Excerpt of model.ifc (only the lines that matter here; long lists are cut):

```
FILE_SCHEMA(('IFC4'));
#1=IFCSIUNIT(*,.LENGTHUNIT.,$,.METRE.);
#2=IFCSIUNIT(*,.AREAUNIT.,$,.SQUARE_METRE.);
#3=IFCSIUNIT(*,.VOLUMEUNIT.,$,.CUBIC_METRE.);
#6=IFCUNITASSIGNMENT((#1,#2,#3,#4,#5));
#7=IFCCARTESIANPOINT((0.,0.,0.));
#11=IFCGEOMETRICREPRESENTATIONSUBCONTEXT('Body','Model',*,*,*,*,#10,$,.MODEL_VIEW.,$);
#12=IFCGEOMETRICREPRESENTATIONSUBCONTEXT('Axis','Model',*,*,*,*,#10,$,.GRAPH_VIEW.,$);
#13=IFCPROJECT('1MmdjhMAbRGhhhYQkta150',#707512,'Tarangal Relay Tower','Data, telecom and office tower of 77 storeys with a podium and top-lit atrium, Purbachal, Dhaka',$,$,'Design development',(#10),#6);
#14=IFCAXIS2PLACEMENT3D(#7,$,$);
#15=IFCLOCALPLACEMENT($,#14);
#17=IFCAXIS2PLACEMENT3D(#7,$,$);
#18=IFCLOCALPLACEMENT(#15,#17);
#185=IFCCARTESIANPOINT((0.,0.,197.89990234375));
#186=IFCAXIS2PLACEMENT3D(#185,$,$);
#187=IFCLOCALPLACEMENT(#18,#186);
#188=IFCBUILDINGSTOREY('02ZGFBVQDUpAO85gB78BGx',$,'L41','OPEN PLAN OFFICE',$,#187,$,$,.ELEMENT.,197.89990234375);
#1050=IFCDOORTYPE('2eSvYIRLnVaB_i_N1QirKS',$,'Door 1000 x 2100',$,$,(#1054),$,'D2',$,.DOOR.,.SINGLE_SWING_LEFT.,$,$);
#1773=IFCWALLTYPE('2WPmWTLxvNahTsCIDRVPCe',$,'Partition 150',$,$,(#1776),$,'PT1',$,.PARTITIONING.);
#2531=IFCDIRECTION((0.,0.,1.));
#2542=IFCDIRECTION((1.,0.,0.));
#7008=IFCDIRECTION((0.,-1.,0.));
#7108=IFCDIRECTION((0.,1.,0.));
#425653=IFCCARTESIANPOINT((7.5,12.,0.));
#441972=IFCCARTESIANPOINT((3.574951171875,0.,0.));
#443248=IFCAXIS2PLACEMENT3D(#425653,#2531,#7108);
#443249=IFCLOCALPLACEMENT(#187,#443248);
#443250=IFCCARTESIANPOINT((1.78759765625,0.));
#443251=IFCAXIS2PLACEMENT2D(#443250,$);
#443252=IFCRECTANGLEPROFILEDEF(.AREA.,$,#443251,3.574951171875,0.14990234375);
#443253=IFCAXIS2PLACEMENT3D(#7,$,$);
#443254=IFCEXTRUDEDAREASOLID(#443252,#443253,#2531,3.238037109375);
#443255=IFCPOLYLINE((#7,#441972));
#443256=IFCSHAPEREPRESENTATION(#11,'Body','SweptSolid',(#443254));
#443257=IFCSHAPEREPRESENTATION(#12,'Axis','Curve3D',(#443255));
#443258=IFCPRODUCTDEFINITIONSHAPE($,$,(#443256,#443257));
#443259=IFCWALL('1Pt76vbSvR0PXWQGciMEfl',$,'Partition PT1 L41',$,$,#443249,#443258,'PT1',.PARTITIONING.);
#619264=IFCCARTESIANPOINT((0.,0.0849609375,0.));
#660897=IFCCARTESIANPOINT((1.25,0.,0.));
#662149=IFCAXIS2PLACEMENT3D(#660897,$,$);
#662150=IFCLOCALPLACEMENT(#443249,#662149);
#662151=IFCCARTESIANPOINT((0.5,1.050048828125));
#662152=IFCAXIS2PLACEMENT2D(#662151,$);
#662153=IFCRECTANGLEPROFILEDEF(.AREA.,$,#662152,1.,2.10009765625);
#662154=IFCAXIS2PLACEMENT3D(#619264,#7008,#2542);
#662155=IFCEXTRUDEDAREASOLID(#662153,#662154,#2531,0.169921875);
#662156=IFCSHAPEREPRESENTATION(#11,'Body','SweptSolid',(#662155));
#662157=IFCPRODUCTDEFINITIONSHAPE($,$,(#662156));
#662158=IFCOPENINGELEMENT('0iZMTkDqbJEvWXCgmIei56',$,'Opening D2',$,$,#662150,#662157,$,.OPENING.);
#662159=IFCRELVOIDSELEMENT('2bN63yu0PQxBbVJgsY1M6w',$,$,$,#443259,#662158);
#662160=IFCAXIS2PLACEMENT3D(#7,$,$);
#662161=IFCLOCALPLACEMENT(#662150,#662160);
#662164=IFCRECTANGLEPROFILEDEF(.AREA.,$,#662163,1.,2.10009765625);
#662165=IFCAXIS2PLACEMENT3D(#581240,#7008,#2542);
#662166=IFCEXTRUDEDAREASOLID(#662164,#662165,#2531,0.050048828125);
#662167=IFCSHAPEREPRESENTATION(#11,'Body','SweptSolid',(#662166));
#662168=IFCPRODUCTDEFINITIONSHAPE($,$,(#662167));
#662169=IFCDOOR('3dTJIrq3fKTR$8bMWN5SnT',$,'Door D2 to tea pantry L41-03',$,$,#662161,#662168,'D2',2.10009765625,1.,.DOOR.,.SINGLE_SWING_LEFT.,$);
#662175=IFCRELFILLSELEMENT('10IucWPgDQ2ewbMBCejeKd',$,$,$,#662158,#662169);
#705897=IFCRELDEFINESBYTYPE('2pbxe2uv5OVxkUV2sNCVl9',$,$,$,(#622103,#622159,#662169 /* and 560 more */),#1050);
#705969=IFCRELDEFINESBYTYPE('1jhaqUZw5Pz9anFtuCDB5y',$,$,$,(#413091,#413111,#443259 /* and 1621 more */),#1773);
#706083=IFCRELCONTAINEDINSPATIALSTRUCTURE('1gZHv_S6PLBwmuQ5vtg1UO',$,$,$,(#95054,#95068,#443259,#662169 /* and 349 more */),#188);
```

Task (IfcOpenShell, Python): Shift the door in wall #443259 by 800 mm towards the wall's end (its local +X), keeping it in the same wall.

```python
import ifcopenshell
import ifcopenshell.api.geometry
import ifcopenshell.util.placement
import ifcopenshell.util.unit

model = ifcopenshell.open("model.ifc")
unit_scale = ifcopenshell.util.unit.calculate_unit_scale(model)

door = model.by_id(662169)
opening = door.FillsVoids[0].RelatingOpeningElement
wall = opening.VoidsElements[0].RelatingBuildingElement

wall_matrix = ifcopenshell.util.placement.get_local_placement(wall.ObjectPlacement)
shift = wall_matrix[:3, 0] * 0.8 / unit_scale
before = ifcopenshell.util.placement.get_local_placement(door.ObjectPlacement)[:3, 3].copy()

# The door is placed relative to its opening, so it follows when the opening moves.
matrix = ifcopenshell.util.placement.get_local_placement(opening.ObjectPlacement)
matrix[:3, 3] += shift
ifcopenshell.api.geometry.edit_object_placement(
    model, product=opening, matrix=matrix, is_si=False, should_transform_children=True
)

after = ifcopenshell.util.placement.get_local_placement(door.ObjectPlacement)[:3, 3]
print("door moved by", (after - before).round(3) + 0.0)

model.write("model-out.ifc")
```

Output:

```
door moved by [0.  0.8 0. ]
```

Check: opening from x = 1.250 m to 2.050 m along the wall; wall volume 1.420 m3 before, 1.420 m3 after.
